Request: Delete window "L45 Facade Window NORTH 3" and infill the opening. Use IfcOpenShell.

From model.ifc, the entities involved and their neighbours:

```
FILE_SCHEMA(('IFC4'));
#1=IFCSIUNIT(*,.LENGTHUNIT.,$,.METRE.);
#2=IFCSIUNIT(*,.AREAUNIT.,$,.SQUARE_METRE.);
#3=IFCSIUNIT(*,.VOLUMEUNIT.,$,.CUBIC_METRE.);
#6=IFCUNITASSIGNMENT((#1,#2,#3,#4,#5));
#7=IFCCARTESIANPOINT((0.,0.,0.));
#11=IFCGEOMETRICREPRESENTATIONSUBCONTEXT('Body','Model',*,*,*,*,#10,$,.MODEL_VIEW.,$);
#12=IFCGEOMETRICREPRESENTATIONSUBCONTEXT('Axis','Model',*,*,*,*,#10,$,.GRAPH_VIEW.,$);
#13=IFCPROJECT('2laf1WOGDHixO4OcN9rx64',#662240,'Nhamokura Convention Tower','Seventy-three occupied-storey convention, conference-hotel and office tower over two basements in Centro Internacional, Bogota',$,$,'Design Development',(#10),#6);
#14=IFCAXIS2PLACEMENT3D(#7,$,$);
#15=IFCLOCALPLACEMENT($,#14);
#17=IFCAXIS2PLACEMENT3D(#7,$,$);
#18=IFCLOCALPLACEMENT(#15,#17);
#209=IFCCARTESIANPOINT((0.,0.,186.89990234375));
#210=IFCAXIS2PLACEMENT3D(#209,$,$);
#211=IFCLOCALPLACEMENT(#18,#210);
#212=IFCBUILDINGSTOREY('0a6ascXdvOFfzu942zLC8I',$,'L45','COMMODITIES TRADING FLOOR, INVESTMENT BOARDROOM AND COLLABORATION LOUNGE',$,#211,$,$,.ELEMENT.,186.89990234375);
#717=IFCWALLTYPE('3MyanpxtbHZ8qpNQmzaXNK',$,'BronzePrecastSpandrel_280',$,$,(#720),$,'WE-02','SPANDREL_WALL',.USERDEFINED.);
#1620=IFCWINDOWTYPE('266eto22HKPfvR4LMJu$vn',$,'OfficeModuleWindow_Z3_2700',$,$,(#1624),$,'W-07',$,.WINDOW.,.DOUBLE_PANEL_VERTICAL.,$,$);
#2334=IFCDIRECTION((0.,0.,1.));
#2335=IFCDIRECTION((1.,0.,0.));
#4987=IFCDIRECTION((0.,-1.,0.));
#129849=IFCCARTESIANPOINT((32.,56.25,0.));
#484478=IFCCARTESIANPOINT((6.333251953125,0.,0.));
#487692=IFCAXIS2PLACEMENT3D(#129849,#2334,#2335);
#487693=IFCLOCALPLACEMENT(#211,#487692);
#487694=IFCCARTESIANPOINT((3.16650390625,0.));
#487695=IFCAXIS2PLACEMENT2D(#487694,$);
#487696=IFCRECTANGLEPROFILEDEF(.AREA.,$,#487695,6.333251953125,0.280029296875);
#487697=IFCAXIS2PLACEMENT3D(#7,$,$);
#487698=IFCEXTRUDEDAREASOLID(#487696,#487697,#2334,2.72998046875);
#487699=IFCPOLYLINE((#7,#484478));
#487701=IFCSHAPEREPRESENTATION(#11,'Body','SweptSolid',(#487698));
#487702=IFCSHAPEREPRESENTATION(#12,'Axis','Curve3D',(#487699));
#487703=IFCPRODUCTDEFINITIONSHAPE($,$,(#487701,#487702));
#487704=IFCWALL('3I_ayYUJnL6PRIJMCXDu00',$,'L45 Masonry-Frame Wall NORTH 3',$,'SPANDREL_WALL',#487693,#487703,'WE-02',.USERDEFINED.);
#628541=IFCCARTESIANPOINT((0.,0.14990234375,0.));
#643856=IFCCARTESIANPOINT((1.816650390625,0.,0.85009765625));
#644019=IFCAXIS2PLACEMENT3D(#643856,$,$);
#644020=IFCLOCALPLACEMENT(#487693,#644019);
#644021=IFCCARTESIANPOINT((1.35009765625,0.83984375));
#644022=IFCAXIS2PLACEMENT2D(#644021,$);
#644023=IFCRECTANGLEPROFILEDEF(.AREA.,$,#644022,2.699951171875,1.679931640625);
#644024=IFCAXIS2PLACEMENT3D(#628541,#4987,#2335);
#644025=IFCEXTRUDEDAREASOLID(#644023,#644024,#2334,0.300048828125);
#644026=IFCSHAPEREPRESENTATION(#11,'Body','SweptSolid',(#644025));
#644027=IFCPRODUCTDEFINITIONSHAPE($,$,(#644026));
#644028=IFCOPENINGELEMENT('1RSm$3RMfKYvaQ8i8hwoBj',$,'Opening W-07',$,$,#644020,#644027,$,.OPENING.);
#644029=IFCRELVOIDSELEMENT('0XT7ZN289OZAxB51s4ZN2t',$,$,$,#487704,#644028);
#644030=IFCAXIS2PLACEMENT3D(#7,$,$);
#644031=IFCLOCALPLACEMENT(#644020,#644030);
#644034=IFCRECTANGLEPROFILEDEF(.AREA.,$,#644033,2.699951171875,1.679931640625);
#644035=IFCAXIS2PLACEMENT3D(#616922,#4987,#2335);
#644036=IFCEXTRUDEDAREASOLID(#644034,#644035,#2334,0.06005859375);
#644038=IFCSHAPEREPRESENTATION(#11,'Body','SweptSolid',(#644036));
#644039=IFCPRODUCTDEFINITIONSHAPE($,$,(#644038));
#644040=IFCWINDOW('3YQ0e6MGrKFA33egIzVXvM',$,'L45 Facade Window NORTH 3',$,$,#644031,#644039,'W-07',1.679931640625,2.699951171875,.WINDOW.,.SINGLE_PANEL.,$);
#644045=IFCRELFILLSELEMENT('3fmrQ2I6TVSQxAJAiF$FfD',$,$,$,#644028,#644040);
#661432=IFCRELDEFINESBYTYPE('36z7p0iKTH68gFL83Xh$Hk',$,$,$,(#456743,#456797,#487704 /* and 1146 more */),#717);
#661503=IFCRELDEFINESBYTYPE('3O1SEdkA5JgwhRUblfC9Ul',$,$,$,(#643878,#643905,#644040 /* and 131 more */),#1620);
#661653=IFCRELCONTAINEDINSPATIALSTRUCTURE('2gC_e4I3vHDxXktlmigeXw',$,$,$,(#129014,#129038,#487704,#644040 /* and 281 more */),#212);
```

```python
import ifcopenshell
import ifcopenshell.api.feature
import ifcopenshell.api.root
import ifcopenshell.geom
import ifcopenshell.util.shape

model = ifcopenshell.open("model.ifc")
settings = ifcopenshell.geom.settings()


def volume(element):
    """Net volume in cubic metres, openings subtracted."""
    shape = ifcopenshell.geom.create_shape(settings, element)
    return ifcopenshell.util.shape.get_volume(shape.geometry)


window = model.by_guid("3YQ0e6MGrKFA33egIzVXvM")
opening = window.FillsVoids[0].RelatingOpeningElement
wall = opening.VoidsElements[0].RelatingBuildingElement
before = volume(wall)

ifcopenshell.api.root.remove_product(model, product=window)
ifcopenshell.api.feature.remove_feature(model, feature=opening)

after = volume(wall)

print(f"wall volume {before:.3f} -> {after:.3f} m3")

model.write("model_updated.ifc")
```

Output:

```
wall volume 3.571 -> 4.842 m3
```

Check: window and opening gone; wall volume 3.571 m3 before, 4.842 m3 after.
